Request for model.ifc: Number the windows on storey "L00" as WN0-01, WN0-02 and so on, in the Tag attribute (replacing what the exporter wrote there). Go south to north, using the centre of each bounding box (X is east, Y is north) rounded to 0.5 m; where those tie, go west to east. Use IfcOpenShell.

First a look at what the model holds.

```python
import ifcopenshell
import ifcopenshell.util.element
import ifcopenshell.util.placement

model = ifcopenshell.open("model.ifc")
print(model.schema)
storey = next(s for s in model.by_type("IfcBuildingStorey") if s.Name == "L00")
windows = [e for e in ifcopenshell.util.element.get_decomposition(storey) if e.is_a("IfcWindow")]
for e in sorted(windows, key=lambda e: e.id()):
    origin = ifcopenshell.util.placement.get_local_placement(e.ObjectPlacement)[:3, 3]
    print(e.id(), e.Tag, e.Name, origin.round(2) + 0.0, sep=" | ")
```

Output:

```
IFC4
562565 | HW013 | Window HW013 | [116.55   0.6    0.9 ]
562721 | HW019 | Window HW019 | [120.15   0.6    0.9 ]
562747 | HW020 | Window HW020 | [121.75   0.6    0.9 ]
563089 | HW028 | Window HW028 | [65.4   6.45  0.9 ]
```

```python
import ifcopenshell
import ifcopenshell.geom
import ifcopenshell.util.element
import ifcopenshell.util.shape

model = ifcopenshell.open("model.ifc")
settings = ifcopenshell.geom.settings()
settings.set("use-world-coords", True)


def centre(element):
    shape = ifcopenshell.geom.create_shape(settings, element)
    return ifcopenshell.util.shape.get_bbox_centroid(shape.geometry)


storey = next(s for s in model.by_type("IfcBuildingStorey") if s.Name == "L00")
windows = [e for e in ifcopenshell.util.element.get_decomposition(storey) if e.is_a("IfcWindow")]

# Insertion points can sit at a corner or the storey origin, so sort by the geometry (in metres).
centres = {e: centre(e) for e in windows}
windows.sort(key=lambda e: (round(centres[e][1] / 0.5), centres[e][0]))

for i, e in enumerate(windows, start=1):
    number = f"WN0-{i:02d}"
    e.Tag = number
    print(e.id(), number)

model.write("model_v2.ifc")
```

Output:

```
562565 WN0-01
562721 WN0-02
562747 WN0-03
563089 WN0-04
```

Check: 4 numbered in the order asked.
